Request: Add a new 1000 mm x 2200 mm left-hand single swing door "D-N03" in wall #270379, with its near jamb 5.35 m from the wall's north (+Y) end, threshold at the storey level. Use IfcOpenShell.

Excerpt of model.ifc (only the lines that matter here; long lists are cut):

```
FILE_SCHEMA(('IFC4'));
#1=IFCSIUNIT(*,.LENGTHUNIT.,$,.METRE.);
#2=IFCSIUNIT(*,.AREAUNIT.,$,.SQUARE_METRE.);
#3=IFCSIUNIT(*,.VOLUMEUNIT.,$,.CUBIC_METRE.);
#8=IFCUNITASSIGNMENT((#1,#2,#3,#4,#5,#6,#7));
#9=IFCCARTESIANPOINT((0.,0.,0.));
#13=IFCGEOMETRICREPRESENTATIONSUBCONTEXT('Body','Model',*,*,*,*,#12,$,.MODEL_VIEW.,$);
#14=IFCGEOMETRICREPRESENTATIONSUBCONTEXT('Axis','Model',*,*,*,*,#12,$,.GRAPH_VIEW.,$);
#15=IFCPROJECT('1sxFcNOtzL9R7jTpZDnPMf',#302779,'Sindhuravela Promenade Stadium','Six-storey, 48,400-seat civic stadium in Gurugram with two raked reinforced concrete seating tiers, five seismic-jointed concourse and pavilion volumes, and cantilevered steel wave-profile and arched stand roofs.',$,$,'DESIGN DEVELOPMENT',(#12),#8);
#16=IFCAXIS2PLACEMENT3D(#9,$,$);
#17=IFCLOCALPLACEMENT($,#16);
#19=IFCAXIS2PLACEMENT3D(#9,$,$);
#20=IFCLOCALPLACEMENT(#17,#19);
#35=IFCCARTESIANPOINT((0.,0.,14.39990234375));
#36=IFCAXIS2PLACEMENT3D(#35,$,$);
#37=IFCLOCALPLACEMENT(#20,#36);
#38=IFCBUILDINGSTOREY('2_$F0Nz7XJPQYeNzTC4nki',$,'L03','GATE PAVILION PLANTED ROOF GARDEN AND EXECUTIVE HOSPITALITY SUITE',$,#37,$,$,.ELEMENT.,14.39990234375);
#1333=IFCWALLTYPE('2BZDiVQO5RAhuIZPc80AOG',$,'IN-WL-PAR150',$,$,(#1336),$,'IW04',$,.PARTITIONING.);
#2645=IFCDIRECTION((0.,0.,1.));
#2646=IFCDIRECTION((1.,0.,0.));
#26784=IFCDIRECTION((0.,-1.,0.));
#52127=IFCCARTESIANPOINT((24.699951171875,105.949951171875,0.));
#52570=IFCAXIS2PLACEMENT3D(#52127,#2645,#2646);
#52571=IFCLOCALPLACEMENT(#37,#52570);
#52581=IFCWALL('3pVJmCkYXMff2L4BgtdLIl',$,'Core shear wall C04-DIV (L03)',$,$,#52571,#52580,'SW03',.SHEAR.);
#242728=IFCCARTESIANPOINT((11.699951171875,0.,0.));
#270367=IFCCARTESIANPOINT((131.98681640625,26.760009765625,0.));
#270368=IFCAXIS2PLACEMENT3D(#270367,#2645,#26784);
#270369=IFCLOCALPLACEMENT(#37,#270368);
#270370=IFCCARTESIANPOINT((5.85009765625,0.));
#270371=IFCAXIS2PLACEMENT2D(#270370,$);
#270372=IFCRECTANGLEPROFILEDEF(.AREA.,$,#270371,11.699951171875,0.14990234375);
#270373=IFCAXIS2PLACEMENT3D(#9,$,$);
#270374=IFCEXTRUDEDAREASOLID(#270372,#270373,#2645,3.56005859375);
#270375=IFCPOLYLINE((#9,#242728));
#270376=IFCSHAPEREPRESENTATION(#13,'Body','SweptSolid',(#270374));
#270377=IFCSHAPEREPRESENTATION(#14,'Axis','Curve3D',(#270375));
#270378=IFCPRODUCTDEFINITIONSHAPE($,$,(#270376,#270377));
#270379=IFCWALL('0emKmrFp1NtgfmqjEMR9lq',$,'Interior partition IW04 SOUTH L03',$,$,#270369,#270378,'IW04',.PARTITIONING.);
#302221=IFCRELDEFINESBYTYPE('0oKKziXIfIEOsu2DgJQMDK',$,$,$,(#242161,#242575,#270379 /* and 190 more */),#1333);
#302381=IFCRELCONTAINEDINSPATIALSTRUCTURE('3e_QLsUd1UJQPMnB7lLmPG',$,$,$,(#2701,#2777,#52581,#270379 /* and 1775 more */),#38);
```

```python
import numpy as np
import ifcopenshell
import ifcopenshell.api.feature
import ifcopenshell.api.geometry
import ifcopenshell.api.root
import ifcopenshell.api.spatial
import ifcopenshell.geom
import ifcopenshell.util.element
import ifcopenshell.util.placement
import ifcopenshell.util.representation
import ifcopenshell.util.shape
import ifcopenshell.util.unit

model = ifcopenshell.open("model.ifc")
unit_scale = ifcopenshell.util.unit.calculate_unit_scale(model)
settings = ifcopenshell.geom.settings()


def volume(element):
    """Net volume in cubic metres, openings subtracted."""
    shape = ifcopenshell.geom.create_shape(settings, element)
    return ifcopenshell.util.shape.get_volume(shape.geometry)


wall = model.by_guid("0emKmrFp1NtgfmqjEMR9lq")
storey = ifcopenshell.util.element.get_container(wall, ifc_class="IfcBuildingStorey")
context = ifcopenshell.util.representation.get_context(model, "Model", "Body", "MODEL_VIEW")
before = volume(wall)

width, height, from_end, sill = 1, 2.2, 5.35, 0.0  # metres

# The wall runs along its own X axis, and the end named is its -X end.
wall_shape = ifcopenshell.geom.create_shape(settings, wall)
x, y, z = ifcopenshell.util.shape.get_vertices(wall_shape.geometry).T
start = x.min() + from_end
face, thickness = float(y.min()), float(y.max() - y.min())
wall_matrix = ifcopenshell.util.placement.get_local_placement(wall.ObjectPlacement)
level = ifcopenshell.util.placement.get_local_placement(storey.ObjectPlacement)[2, 3]


def in_wall(x, y):
    """Placement at x, y metres in the wall's axes, at sill height."""
    matrix = wall_matrix.copy()
    matrix[:, 3] = wall_matrix @ np.array([x / unit_scale, y / unit_scale, 0.0, 1.0])
    matrix[2, 3] = level + sill / unit_scale
    return matrix


# Opening: a box that overshoots both wall faces by 50 mm.
opening = ifcopenshell.api.root.create_entity(model, ifc_class="IfcOpeningElement", predefined_type="OPENING")
box = ifcopenshell.api.geometry.add_wall_representation(
    model, context=context, length=width, height=height, thickness=thickness + 0.1
)
ifcopenshell.api.geometry.assign_representation(model, product=opening, representation=box)
ifcopenshell.api.geometry.edit_object_placement(model, product=opening, matrix=in_wall(start, face - 0.05), is_si=False)
ifcopenshell.api.feature.add_feature(model, feature=opening, element=wall)

door = ifcopenshell.api.root.create_entity(model, ifc_class="IfcDoor", name="D-N03", predefined_type="DOOR")
door.OverallWidth, door.OverallHeight = width / unit_scale, height / unit_scale
door.OperationType = "SINGLE_SWING_LEFT"
body = ifcopenshell.api.geometry.add_door_representation(
    model,
    context=context,
    overall_width=door.OverallWidth,
    overall_height=door.OverallHeight,
    operation_type="SINGLE_SWING_LEFT",
    lining_properties={"LiningDepth": thickness / unit_scale, "ThresholdDepth": thickness / unit_scale},
)
ifcopenshell.api.geometry.assign_representation(model, product=door, representation=body)
ifcopenshell.api.spatial.assign_container(model, products=[door], relating_structure=storey)
ifcopenshell.api.feature.add_filling(model, opening=opening, element=door)

# The lining spans the wall, so the door starts at the wall face.
ifcopenshell.api.geometry.edit_object_placement(model, product=door, matrix=in_wall(start, face), is_si=False)

after = volume(wall)

print(f"wall volume {before:.3f} -> {after:.3f} m3")

model.write("model_updated.ifc")
```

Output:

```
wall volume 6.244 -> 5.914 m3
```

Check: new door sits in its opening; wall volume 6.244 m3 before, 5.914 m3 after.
